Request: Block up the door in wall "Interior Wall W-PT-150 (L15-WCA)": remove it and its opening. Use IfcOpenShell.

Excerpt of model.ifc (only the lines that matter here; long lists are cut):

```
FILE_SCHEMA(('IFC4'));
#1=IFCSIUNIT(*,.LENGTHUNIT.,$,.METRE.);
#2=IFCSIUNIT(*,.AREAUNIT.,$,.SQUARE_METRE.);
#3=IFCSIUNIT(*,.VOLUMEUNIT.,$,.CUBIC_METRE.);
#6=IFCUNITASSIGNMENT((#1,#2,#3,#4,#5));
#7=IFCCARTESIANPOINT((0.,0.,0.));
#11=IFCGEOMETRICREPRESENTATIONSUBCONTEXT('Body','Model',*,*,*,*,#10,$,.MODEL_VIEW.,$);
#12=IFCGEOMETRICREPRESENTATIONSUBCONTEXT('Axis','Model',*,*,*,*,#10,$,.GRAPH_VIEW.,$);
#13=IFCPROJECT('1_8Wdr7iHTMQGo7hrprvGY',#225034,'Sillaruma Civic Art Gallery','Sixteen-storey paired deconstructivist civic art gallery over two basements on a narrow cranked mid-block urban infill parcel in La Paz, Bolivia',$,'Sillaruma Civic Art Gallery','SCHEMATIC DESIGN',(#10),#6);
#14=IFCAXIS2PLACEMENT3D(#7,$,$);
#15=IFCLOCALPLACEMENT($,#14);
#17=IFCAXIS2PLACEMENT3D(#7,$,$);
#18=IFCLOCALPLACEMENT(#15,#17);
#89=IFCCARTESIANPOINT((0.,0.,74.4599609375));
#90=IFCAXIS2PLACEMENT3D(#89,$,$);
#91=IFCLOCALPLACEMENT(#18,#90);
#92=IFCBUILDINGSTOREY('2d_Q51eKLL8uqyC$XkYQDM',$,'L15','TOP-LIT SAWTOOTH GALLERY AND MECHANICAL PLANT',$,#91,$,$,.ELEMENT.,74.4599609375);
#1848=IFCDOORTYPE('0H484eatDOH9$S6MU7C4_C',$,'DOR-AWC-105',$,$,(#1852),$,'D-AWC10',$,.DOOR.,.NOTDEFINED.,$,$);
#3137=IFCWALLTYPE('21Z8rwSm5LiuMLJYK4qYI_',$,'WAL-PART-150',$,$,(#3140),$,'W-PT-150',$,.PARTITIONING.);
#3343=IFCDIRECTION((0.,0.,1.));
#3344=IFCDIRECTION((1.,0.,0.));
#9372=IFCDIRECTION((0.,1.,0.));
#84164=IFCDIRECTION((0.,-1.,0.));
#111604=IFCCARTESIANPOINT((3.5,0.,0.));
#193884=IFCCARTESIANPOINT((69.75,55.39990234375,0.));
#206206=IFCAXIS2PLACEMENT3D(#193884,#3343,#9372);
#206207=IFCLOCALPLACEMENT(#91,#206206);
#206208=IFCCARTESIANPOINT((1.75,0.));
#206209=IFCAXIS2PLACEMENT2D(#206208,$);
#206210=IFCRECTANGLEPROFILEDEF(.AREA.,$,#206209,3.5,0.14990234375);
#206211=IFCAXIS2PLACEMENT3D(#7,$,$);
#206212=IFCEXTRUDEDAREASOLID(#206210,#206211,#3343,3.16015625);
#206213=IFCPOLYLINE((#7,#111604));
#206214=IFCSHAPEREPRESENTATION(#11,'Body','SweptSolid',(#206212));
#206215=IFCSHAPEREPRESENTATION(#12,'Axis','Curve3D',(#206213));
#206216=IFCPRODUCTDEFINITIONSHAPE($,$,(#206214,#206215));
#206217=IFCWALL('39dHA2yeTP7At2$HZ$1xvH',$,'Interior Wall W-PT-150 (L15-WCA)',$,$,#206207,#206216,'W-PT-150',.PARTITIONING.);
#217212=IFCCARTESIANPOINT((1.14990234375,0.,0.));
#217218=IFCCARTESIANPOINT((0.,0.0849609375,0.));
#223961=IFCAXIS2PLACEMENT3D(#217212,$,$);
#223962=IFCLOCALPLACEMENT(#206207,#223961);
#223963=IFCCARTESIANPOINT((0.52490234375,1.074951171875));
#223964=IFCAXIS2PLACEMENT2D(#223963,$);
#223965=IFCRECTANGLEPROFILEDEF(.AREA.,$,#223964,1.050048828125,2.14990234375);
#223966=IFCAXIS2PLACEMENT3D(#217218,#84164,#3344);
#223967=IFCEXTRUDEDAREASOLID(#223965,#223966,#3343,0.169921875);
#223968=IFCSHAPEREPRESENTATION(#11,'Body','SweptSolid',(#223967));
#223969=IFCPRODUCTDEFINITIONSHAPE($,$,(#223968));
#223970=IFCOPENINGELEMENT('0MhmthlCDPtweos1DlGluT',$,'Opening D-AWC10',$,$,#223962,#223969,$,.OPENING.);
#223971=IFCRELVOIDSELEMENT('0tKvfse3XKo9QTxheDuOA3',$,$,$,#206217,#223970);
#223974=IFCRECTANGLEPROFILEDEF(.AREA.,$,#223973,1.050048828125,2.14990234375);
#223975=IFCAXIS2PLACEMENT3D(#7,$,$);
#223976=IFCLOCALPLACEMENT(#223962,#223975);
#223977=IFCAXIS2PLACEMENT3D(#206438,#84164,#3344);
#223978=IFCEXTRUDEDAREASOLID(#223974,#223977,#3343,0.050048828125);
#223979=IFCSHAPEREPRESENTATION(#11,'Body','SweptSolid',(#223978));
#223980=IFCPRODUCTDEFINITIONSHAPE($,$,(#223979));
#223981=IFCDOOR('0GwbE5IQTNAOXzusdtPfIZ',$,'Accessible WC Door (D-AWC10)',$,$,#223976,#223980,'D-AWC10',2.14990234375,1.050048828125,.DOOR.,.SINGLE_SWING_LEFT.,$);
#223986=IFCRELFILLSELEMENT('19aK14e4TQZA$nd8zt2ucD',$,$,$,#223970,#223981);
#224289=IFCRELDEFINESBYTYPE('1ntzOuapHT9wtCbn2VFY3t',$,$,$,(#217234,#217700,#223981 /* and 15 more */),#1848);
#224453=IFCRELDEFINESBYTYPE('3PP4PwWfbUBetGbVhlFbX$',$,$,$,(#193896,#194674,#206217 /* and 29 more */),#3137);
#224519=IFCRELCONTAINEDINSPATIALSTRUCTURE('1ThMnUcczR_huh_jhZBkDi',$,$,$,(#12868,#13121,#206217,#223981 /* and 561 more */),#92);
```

```python
import ifcopenshell
import ifcopenshell.api.feature
import ifcopenshell.api.root
import ifcopenshell.geom
import ifcopenshell.util.shape

model = ifcopenshell.open("model.ifc")
settings = ifcopenshell.geom.settings()


def volume(element):
    """Net volume in cubic metres, openings subtracted."""
    shape = ifcopenshell.geom.create_shape(settings, element)
    return ifcopenshell.util.shape.get_volume(shape.geometry)


door = model.by_guid("0GwbE5IQTNAOXzusdtPfIZ")
opening = door.FillsVoids[0].RelatingOpeningElement
wall = opening.VoidsElements[0].RelatingBuildingElement
before = volume(wall)

ifcopenshell.api.root.remove_product(model, product=door)
ifcopenshell.api.feature.remove_feature(model, feature=opening)

after = volume(wall)

print(f"wall volume {before:.3f} -> {after:.3f} m3")

model.write("model_rev.ifc")
```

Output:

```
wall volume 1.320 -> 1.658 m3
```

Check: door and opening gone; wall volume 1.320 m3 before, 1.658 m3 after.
